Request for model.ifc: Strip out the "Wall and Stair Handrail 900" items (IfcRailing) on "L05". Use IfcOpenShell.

First a look at what the model holds.

```python
import ifcopenshell
import ifcopenshell.util.element

model = ifcopenshell.open("model.ifc")
print(model.schema)
storey = next(s for s in model.by_type("IfcBuildingStorey") if s.Name == "L05")
railings = [e for e in ifcopenshell.util.element.get_decomposition(storey) if e.is_a("IfcRailing")]
seen = {}
for e in railings:
    element_type = ifcopenshell.util.element.get_type(e)
    name = element_type.Name if element_type not in (None, e) else None
    seen[name] = seen.get(name, 0) + 1
for name, count in sorted(seen.items(), key=str):
    print(count, "x", name)
```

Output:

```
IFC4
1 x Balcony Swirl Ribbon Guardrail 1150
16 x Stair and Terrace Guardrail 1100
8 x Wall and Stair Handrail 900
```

```python
import ifcopenshell
import ifcopenshell.api.root
import ifcopenshell.util.element

model = ifcopenshell.open("model.ifc")

storey = next(s for s in model.by_type("IfcBuildingStorey") if s.Name == "L05")
railings = [e for e in ifcopenshell.util.element.get_decomposition(storey) if e.is_a("IfcRailing")]
targets = [e for e in railings if (t := ifcopenshell.util.element.get_type(e)) not in (None, e) and t.Name == "Wall and Stair Handrail 900"]

for e in targets:
    ifcopenshell.api.root.remove_product(model, product=e)
print(len(targets), "removed")

model.write("model_edited.ifc")
```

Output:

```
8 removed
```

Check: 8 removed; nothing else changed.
